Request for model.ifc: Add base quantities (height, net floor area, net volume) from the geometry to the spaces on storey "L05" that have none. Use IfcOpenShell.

First a look at what the model holds.

```python
import ifcopenshell
import ifcopenshell.util.element
import ifcopenshell.util.unit

model = ifcopenshell.open("model.ifc")
print(model.schema)
for unit_type in ("LENGTHUNIT", "AREAUNIT", "VOLUMEUNIT"):
    print(unit_type, ifcopenshell.util.unit.calculate_unit_scale(model, unit_type))
storey = next(s for s in model.by_type("IfcBuildingStorey") if s.Name == "L05")
spaces = [e for e in ifcopenshell.util.element.get_decomposition(storey) if e.is_a("IfcSpace")]
for e in sorted(spaces, key=lambda e: e.id()):
    print(e.id(), e.is_a(), e.Name, list(ifcopenshell.util.element.get_psets(e, qtos_only=True)), sep=" | ")
```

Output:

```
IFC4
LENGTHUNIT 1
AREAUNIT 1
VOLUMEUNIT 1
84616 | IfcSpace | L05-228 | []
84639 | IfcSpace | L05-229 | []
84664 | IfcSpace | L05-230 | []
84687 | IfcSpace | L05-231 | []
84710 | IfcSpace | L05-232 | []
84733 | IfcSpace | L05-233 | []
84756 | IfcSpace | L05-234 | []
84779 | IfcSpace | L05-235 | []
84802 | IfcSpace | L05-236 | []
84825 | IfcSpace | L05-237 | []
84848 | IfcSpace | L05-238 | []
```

```python
import ifcopenshell
import ifcopenshell.api.pset
import ifcopenshell.geom
import ifcopenshell.util.element
import ifcopenshell.util.shape
import ifcopenshell.util.unit

model = ifcopenshell.open("model.ifc")
unit_scale = ifcopenshell.util.unit.calculate_unit_scale(model)
area_scale = ifcopenshell.util.unit.calculate_unit_scale(model, "AREAUNIT")
volume_scale = ifcopenshell.util.unit.calculate_unit_scale(model, "VOLUMEUNIT")
settings = ifcopenshell.geom.settings()

storey = next(s for s in model.by_type("IfcBuildingStorey") if s.Name == "L05")
spaces = [e for e in ifcopenshell.util.element.get_decomposition(storey) if e.is_a("IfcSpace")]

for e in sorted(spaces, key=lambda e: e.id()):
    if ifcopenshell.util.element.get_psets(e, qtos_only=True, should_inherit=False):
        continue
    # Geometry comes back in metres, in the element's own axes.
    shape = ifcopenshell.geom.create_shape(settings, e)
    values = {
        "Height": ifcopenshell.util.shape.get_z(shape.geometry) / unit_scale,
        "NetFloorArea": ifcopenshell.util.shape.get_footprint_area(shape.geometry) / area_scale,
        "NetVolume": ifcopenshell.util.shape.get_volume(shape.geometry) / volume_scale,
    }
    qto = ifcopenshell.api.pset.add_qto(model, product=e, name="Qto_SpaceBaseQuantities")
    ifcopenshell.api.pset.edit_qto(model, qto=qto, properties=values)
    print(e.id(), {k: round(v, 3) for k, v in values.items()})

model.write("model_v2.ifc")
```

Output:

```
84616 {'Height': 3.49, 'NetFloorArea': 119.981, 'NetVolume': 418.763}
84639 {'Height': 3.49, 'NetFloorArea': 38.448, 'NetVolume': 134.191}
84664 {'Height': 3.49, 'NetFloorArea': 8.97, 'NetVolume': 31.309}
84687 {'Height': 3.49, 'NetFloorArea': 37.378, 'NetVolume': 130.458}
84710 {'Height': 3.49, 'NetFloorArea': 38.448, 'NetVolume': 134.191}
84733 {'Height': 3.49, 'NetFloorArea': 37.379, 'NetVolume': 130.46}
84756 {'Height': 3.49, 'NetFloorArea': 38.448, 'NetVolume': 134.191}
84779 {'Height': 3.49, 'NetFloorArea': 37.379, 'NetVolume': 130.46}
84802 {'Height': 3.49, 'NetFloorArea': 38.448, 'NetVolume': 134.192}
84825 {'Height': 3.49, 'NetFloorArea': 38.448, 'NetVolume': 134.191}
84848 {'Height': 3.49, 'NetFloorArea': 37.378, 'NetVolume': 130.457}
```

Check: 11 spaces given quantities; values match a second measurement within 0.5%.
